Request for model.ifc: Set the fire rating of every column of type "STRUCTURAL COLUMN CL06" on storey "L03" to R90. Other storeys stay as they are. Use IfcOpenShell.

First a look at what the model holds.

```python
import ifcopenshell
import ifcopenshell.util.element

model = ifcopenshell.open("model.ifc")
print(model.schema)
storey = next(s for s in model.by_type("IfcBuildingStorey") if s.Name == "L03")
columns = [e for e in ifcopenshell.util.element.get_decomposition(storey) if e.is_a("IfcColumn")]
seen = {}
for e in columns:
    element_type = ifcopenshell.util.element.get_type(e)
    key = (element_type.Name if element_type != e and element_type else None, ifcopenshell.util.element.get_pset(e, "Pset_ColumnCommon", "FireRating"))
    seen[key] = seen.get(key, 0) + 1
for (name, value), count in sorted(seen.items(), key=str):
    print(count, "x", name, "|", value)
```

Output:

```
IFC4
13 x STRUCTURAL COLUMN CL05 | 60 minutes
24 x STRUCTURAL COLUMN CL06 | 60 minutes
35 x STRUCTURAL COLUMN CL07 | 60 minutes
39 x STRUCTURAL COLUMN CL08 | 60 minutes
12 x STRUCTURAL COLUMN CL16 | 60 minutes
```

```python
import ifcopenshell
import ifcopenshell.api.pset
import ifcopenshell.util.element

model = ifcopenshell.open("model.ifc")

storey = next(s for s in model.by_type("IfcBuildingStorey") if s.Name == "L03")
columns = [e for e in ifcopenshell.util.element.get_decomposition(storey) if e.is_a("IfcColumn")]

count = 0
for e in columns:
    element_type = ifcopenshell.util.element.get_type(e)
    if element_type in (None, e) or element_type.Name != "STRUCTURAL COLUMN CL06":
        continue
    # add_pset returns the element's existing set when there is one.
    pset = ifcopenshell.api.pset.add_pset(model, product=e, name="Pset_ColumnCommon")
    ifcopenshell.api.pset.edit_pset(model, pset=pset, properties={"FireRating": "R90"})
    count += 1

print(count, "columns updated")

model.write("model-out.ifc")
```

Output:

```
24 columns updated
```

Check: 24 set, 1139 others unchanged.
